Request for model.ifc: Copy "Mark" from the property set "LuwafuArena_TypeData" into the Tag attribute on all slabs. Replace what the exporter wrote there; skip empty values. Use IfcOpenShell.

First a look at what the model holds.

```python
import ifcopenshell
import ifcopenshell.util.element

model = ifcopenshell.open("model.ifc")
print(model.schema)
slabs = model.by_type("IfcSlab")
print(len(slabs), "slabs")
for e in slabs[:8]:
    source = ifcopenshell.util.element.get_pset(e, "LuwafuArena_TypeData", "Mark")
    target = e.Tag
    print(e.id(), repr(source), repr(target), sep=" | ")
```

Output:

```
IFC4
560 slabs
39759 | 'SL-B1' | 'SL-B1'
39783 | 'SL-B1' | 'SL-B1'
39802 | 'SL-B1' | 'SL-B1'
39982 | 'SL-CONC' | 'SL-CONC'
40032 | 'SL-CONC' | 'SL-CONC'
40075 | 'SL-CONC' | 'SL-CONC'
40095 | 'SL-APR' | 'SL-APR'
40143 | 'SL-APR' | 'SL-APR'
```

```python
import ifcopenshell
import ifcopenshell.util.element

model = ifcopenshell.open("model.ifc")

count = 0
for e in model.by_type("IfcSlab"):
    value = ifcopenshell.util.element.get_pset(e, "LuwafuArena_TypeData", "Mark")
    current = e.Tag
    if not value or not value.strip() or current == value:
        continue
    e.Tag = value
    count += 1

print(count, "slabs updated")

model.write("model_edited.ifc")
```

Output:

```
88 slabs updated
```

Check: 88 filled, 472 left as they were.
